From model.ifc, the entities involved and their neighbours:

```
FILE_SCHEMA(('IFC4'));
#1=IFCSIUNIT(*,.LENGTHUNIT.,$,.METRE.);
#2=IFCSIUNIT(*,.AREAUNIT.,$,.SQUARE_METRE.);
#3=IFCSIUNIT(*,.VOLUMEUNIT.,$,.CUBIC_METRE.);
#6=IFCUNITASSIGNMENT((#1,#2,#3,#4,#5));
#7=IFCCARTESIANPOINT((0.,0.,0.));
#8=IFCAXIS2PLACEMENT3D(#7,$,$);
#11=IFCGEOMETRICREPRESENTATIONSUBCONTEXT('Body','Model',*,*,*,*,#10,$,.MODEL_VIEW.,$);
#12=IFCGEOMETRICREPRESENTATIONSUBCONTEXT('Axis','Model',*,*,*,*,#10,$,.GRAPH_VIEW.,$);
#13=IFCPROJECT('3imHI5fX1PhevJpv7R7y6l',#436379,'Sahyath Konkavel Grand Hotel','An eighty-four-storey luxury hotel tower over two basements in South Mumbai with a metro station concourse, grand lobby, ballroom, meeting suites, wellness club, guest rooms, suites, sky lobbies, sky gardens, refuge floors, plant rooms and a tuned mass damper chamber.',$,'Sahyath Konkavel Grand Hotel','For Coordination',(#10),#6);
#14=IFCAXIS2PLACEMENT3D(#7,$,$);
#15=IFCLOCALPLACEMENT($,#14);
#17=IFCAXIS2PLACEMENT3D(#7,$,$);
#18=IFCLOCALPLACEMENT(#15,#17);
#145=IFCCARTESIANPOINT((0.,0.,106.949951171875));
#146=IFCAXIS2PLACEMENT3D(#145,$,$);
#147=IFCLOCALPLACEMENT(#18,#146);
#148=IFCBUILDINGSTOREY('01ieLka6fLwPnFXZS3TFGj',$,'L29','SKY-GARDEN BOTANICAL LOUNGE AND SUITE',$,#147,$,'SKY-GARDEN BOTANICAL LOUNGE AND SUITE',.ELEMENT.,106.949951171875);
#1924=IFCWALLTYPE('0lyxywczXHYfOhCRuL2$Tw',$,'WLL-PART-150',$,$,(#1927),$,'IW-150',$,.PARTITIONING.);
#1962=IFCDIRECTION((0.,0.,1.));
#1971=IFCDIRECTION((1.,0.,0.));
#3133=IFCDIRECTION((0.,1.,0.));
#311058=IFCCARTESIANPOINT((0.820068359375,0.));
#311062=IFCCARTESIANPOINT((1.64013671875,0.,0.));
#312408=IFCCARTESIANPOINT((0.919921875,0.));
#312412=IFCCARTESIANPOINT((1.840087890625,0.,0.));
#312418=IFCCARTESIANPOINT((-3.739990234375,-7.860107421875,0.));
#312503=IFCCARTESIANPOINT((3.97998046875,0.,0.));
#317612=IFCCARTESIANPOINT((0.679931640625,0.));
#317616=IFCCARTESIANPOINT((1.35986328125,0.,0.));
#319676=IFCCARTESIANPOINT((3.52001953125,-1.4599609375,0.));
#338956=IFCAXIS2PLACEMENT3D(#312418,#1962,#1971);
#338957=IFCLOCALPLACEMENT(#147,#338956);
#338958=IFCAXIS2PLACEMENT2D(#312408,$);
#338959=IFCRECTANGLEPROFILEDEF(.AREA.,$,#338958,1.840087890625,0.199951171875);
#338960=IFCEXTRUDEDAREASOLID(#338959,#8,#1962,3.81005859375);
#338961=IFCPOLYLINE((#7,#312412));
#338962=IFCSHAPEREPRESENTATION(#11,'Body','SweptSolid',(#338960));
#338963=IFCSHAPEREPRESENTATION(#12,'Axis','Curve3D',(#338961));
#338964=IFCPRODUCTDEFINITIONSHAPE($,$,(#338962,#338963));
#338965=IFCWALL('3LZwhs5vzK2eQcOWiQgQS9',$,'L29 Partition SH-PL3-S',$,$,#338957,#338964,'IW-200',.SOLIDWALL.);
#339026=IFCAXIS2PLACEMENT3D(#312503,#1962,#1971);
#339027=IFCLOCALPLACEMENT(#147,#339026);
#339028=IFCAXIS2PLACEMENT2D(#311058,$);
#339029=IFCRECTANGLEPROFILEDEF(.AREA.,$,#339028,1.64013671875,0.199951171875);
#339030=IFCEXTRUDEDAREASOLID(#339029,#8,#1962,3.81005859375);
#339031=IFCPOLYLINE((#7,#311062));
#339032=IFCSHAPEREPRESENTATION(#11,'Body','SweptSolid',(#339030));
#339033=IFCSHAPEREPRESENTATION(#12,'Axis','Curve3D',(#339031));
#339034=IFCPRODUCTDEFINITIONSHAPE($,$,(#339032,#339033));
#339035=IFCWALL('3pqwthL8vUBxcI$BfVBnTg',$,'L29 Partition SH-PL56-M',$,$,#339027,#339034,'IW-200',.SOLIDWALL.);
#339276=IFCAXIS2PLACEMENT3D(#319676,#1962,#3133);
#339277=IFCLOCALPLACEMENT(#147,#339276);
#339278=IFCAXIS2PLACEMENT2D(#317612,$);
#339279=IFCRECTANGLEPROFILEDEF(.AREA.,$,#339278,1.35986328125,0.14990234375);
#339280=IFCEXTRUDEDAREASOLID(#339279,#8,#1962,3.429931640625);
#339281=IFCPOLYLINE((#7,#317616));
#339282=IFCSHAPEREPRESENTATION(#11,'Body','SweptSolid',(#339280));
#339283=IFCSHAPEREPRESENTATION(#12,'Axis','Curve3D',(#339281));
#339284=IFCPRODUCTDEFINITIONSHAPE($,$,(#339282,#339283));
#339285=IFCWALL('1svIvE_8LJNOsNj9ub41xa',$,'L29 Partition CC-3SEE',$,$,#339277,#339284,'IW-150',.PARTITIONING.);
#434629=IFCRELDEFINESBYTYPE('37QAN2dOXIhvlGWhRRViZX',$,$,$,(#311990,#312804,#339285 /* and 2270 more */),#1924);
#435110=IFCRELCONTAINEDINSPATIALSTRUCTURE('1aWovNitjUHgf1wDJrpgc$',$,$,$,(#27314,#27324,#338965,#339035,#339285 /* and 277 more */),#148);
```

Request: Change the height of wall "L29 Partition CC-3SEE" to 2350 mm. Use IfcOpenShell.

```python
import ifcopenshell
import ifcopenshell.geom
import ifcopenshell.util.representation
import ifcopenshell.util.shape
import ifcopenshell.util.unit

model = ifcopenshell.open("model.ifc")
unit_scale = ifcopenshell.util.unit.calculate_unit_scale(model)
settings = ifcopenshell.geom.settings()


def volume(element):
    """Net volume in cubic metres, openings subtracted."""
    shape = ifcopenshell.geom.create_shape(settings, element)
    return ifcopenshell.util.shape.get_volume(shape.geometry)


wall = model.by_guid("1svIvE_8LJNOsNj9ub41xa")
before = volume(wall)

body = ifcopenshell.util.representation.get_representation(wall, "Model", "Body")
solid = body.Items[0]
old_height = solid.Depth
solid.Depth = 2.35 / unit_scale
after = volume(wall)

print(f"height {old_height:g} -> {solid.Depth:g}, volume {before:.3f} -> {after:.3f} m3")

model.write("model_rev.ifc")
```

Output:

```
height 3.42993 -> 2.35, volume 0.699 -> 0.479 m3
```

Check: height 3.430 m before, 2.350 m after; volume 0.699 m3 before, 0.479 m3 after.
